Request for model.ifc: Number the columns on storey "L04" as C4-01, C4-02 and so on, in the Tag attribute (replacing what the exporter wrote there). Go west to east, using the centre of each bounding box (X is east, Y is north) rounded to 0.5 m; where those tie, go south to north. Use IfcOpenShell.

First a look at what the model holds.

```python
import ifcopenshell
import ifcopenshell.util.element
import ifcopenshell.util.placement

model = ifcopenshell.open("model.ifc")
print(model.schema)
storey = next(s for s in model.by_type("IfcBuildingStorey") if s.Name == "L04")
columns = [e for e in ifcopenshell.util.element.get_decomposition(storey) if e.is_a("IfcColumn")]
for e in sorted(columns, key=lambda e: e.id()):
    origin = ifcopenshell.util.placement.get_local_placement(e.ObjectPlacement)[:3, 3]
    print(e.id(), e.Tag, e.Name, origin.round(2) + 0.0, sep=" | ")
```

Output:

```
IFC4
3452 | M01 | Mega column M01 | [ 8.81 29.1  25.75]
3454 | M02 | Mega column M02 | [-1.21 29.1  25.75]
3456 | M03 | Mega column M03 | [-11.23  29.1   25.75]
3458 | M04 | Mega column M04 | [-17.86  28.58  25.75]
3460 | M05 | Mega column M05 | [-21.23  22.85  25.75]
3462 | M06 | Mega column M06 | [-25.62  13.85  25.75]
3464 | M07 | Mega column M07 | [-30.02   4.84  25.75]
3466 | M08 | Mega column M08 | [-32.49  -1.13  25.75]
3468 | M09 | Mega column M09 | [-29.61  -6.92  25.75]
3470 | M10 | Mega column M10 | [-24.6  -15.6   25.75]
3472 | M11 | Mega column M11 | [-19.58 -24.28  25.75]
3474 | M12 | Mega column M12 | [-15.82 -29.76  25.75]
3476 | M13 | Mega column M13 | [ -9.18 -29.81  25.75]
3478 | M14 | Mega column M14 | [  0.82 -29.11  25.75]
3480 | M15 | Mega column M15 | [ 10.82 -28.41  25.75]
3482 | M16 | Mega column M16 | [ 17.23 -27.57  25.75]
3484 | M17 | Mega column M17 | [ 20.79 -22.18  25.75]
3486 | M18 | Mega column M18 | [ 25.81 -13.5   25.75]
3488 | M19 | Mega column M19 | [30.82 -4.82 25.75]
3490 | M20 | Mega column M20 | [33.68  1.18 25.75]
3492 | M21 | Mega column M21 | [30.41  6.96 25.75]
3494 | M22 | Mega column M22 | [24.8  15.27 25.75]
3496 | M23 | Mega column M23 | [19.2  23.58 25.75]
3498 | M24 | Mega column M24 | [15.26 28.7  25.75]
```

```python
import ifcopenshell
import ifcopenshell.geom
import ifcopenshell.util.element
import ifcopenshell.util.shape

model = ifcopenshell.open("model.ifc")
settings = ifcopenshell.geom.settings()
settings.set("use-world-coords", True)


def centre(element):
    shape = ifcopenshell.geom.create_shape(settings, element)
    return ifcopenshell.util.shape.get_bbox_centroid(shape.geometry)


storey = next(s for s in model.by_type("IfcBuildingStorey") if s.Name == "L04")
columns = [e for e in ifcopenshell.util.element.get_decomposition(storey) if e.is_a("IfcColumn")]

# Insertion points can sit at a corner or the storey origin, so sort by the geometry (in metres).
centres = {e: centre(e) for e in columns}
columns.sort(key=lambda e: (round(centres[e][0] / 0.5), centres[e][1]))

for i, e in enumerate(columns, start=1):
    number = f"C4-{i:02d}"
    e.Tag = number
    print(e.id(), number)

model.write("model_rev.ifc")
```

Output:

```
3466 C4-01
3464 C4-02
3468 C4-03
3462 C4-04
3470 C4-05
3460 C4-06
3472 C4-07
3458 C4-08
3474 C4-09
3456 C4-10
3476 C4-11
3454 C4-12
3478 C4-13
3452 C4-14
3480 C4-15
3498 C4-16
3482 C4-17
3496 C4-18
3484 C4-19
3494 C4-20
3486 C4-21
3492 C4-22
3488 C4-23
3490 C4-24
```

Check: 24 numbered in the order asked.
